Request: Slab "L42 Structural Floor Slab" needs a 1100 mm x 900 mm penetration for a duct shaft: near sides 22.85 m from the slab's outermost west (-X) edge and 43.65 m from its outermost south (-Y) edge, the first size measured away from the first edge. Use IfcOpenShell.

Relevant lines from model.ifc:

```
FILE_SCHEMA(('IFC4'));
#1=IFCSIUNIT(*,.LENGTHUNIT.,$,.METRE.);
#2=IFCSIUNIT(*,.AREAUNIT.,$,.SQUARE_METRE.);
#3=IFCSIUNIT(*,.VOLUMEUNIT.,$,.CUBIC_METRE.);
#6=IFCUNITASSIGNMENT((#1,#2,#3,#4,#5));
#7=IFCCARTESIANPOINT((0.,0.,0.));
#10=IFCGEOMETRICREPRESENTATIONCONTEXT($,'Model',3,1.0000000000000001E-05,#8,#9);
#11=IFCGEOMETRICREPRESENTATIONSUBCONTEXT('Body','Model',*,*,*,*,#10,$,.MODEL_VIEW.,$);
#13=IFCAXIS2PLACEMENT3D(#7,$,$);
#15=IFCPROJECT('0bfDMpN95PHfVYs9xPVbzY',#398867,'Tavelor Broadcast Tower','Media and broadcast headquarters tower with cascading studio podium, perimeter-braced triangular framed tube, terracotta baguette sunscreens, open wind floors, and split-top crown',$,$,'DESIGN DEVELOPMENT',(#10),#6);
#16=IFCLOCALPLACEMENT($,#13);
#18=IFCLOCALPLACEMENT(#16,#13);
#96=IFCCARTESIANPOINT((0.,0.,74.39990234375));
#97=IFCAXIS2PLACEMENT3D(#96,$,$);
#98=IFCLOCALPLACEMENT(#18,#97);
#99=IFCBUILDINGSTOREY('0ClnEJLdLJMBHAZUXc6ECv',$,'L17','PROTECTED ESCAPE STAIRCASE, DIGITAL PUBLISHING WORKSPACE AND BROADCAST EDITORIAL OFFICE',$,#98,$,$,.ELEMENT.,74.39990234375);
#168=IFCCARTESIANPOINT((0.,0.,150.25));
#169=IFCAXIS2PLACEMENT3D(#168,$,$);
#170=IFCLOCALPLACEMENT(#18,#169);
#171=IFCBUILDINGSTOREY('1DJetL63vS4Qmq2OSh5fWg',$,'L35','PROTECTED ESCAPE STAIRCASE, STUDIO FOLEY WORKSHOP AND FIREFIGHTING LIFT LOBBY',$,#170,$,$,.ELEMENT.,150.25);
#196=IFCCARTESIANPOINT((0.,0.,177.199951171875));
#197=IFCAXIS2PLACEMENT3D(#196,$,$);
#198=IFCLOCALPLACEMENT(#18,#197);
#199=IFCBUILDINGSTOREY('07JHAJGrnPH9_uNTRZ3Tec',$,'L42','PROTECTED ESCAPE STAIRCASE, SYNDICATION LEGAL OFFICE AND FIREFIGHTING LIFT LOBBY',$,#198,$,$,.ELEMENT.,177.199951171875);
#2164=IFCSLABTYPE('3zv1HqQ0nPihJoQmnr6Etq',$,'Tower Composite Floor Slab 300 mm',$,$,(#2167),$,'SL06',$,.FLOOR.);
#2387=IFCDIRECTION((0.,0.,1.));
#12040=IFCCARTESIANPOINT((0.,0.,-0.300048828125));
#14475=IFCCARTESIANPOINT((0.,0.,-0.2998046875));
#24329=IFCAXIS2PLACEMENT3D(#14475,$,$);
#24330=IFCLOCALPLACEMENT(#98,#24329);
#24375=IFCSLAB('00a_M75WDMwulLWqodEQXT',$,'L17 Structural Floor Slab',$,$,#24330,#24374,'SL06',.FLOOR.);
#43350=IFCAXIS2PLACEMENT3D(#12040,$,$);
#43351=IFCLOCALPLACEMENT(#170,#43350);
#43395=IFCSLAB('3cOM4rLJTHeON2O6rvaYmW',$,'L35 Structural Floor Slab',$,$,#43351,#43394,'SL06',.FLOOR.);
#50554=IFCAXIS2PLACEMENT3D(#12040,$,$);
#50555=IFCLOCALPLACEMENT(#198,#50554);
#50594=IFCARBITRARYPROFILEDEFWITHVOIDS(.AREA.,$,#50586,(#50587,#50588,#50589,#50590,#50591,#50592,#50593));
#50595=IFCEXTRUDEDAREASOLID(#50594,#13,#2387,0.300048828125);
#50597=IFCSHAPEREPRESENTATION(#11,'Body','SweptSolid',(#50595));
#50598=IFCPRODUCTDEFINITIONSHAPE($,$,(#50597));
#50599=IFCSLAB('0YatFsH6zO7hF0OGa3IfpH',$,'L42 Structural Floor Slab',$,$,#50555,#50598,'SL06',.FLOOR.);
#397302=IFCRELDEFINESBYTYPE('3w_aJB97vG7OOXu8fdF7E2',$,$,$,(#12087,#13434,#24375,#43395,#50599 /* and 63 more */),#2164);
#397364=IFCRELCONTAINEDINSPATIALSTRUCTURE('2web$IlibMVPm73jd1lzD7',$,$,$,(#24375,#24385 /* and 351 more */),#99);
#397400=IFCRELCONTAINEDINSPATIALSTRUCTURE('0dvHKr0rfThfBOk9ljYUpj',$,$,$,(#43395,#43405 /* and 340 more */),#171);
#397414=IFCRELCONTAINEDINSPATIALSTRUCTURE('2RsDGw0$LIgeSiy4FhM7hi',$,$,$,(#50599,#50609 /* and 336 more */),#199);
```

```python
import numpy as np
import ifcopenshell
import ifcopenshell.api.feature
import ifcopenshell.api.geometry
import ifcopenshell.api.root
import ifcopenshell.geom
import ifcopenshell.util.placement
import ifcopenshell.util.representation
import ifcopenshell.util.shape
import ifcopenshell.util.unit

model = ifcopenshell.open("model.ifc")
unit_scale = ifcopenshell.util.unit.calculate_unit_scale(model)
settings = ifcopenshell.geom.settings()


def volume(element):
    """Net volume in cubic metres, openings subtracted."""
    shape = ifcopenshell.geom.create_shape(settings, element)
    return ifcopenshell.util.shape.get_volume(shape.geometry)


slab = model.by_guid("0YatFsH6zO7hF0OGa3IfpH")
before = volume(slab)

# Extent in the slab's own axes, in metres. The edges named are its -X and -Y sides.
slab_shape = ifcopenshell.geom.create_shape(settings, slab)
vertices = ifcopenshell.util.shape.get_vertices(slab_shape.geometry)
x_min, y_min, bottom = vertices.min(axis=0)
top = vertices[:, 2].max()

opening = ifcopenshell.api.root.create_entity(model, ifc_class="IfcOpeningElement", name="Duct shaft opening", predefined_type="OPENING")
context = ifcopenshell.util.representation.get_context(model, "Model", "Body", "MODEL_VIEW")
width, depth = 1.1, 0.9
outline = [(0.0, 0.0), (width, 0.0), (width, depth), (0.0, depth), (0.0, 0.0)]
# Overshoot both faces by 50 mm so the cut is clean.
shape = ifcopenshell.api.geometry.add_slab_representation(
    model, context=context, depth=top - bottom + 0.1, polyline=outline
)
ifcopenshell.api.geometry.assign_representation(model, product=opening, representation=shape)

matrix = ifcopenshell.util.placement.get_local_placement(slab.ObjectPlacement)
matrix[:, 3] = matrix @ np.append(np.array([x_min + 22.85, y_min + 43.65, bottom - 0.05]) / unit_scale, 1.0)
ifcopenshell.api.geometry.edit_object_placement(model, product=opening, matrix=matrix, is_si=False)
ifcopenshell.api.feature.add_feature(model, feature=opening, element=slab)

after = volume(slab)

print(f"slab volume {before:.3f} -> {after:.3f} m3")

model.write("model_v2.ifc")
```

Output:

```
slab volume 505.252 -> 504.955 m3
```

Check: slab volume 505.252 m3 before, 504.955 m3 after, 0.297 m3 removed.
